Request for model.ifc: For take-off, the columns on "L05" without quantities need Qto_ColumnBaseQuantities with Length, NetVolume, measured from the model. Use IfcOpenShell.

First a look at what the model holds.

```python
import ifcopenshell
import ifcopenshell.util.element
import ifcopenshell.util.unit

model = ifcopenshell.open("model.ifc")
print(model.schema)
for unit_type in ("LENGTHUNIT", "AREAUNIT", "VOLUMEUNIT"):
    print(unit_type, ifcopenshell.util.unit.calculate_unit_scale(model, unit_type))
storey = next(s for s in model.by_type("IfcBuildingStorey") if s.Name == "L05")
columns = [e for e in ifcopenshell.util.element.get_decomposition(storey) if e.is_a("IfcColumn")]
for e in sorted(columns, key=lambda e: e.id()):
    print(e.id(), e.is_a(), e.Name, list(ifcopenshell.util.element.get_psets(e, qtos_only=True)), sep=" | ")
```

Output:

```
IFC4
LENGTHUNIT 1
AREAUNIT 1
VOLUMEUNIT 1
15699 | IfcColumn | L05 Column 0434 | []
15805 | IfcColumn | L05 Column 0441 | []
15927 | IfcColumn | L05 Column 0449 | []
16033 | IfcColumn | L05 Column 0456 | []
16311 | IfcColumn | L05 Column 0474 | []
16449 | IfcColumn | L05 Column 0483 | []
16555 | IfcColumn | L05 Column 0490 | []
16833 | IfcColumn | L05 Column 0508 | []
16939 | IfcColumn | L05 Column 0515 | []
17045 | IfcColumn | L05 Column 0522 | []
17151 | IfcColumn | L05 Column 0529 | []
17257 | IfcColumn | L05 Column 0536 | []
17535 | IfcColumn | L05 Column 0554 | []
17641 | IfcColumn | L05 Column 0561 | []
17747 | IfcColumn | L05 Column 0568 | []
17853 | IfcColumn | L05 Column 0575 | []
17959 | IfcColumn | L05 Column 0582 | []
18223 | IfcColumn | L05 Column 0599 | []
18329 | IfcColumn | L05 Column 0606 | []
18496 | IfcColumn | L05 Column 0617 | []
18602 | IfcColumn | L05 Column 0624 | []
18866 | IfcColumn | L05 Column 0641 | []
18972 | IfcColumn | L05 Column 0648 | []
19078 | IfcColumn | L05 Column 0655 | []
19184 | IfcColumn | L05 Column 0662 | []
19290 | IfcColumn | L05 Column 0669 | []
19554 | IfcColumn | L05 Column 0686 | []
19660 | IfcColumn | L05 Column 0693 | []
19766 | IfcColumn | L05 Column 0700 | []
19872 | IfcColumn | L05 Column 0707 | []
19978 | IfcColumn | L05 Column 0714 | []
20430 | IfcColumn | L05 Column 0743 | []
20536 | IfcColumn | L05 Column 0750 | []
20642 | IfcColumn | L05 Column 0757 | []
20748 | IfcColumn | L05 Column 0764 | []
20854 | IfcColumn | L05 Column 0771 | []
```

```python
import ifcopenshell
import ifcopenshell.api.pset
import ifcopenshell.geom
import ifcopenshell.util.element
import ifcopenshell.util.shape
import ifcopenshell.util.unit

model = ifcopenshell.open("model.ifc")
unit_scale = ifcopenshell.util.unit.calculate_unit_scale(model)
volume_scale = ifcopenshell.util.unit.calculate_unit_scale(model, "VOLUMEUNIT")
settings = ifcopenshell.geom.settings()

storey = next(s for s in model.by_type("IfcBuildingStorey") if s.Name == "L05")
columns = [e for e in ifcopenshell.util.element.get_decomposition(storey) if e.is_a("IfcColumn")]

for e in sorted(columns, key=lambda e: e.id()):
    if ifcopenshell.util.element.get_psets(e, qtos_only=True, should_inherit=False):
        continue
    # Geometry comes back in metres, in the element's own axes.
    shape = ifcopenshell.geom.create_shape(settings, e)
    values = {
        "Length": ifcopenshell.util.shape.get_z(shape.geometry) / unit_scale,
        "NetVolume": ifcopenshell.util.shape.get_volume(shape.geometry) / volume_scale,
    }
    qto = ifcopenshell.api.pset.add_qto(model, product=e, name="Qto_ColumnBaseQuantities")
    ifcopenshell.api.pset.edit_qto(model, qto=qto, properties=values)
    print(e.id(), {k: round(v, 3) for k, v in values.items()})

model.write("model_updated.ifc")
```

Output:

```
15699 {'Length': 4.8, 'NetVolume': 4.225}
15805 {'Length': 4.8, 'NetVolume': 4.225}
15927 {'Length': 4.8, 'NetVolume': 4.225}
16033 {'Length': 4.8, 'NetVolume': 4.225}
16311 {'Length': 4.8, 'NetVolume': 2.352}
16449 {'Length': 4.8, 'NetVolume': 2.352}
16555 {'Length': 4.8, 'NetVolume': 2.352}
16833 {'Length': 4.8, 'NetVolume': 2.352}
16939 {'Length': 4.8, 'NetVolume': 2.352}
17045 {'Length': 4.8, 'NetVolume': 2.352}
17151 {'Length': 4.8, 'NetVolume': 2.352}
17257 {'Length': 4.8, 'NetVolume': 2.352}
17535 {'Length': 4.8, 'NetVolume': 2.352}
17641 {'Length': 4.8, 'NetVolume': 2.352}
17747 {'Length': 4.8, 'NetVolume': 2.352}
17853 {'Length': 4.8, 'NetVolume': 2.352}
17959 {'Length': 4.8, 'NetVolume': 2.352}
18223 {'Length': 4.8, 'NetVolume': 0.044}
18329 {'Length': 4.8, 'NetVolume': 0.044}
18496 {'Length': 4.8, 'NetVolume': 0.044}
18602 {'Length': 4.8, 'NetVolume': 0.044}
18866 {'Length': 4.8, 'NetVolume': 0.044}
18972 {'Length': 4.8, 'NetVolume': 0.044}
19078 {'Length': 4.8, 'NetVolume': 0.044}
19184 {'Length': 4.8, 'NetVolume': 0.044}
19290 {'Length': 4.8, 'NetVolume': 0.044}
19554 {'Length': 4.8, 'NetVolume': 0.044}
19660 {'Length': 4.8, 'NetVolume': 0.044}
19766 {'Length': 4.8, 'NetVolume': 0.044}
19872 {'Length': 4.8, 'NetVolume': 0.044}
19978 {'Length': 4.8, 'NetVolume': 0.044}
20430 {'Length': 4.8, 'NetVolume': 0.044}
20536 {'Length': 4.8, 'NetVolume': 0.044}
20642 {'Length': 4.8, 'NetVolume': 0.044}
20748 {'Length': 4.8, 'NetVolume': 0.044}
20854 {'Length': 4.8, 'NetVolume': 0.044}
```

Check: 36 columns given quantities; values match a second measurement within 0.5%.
